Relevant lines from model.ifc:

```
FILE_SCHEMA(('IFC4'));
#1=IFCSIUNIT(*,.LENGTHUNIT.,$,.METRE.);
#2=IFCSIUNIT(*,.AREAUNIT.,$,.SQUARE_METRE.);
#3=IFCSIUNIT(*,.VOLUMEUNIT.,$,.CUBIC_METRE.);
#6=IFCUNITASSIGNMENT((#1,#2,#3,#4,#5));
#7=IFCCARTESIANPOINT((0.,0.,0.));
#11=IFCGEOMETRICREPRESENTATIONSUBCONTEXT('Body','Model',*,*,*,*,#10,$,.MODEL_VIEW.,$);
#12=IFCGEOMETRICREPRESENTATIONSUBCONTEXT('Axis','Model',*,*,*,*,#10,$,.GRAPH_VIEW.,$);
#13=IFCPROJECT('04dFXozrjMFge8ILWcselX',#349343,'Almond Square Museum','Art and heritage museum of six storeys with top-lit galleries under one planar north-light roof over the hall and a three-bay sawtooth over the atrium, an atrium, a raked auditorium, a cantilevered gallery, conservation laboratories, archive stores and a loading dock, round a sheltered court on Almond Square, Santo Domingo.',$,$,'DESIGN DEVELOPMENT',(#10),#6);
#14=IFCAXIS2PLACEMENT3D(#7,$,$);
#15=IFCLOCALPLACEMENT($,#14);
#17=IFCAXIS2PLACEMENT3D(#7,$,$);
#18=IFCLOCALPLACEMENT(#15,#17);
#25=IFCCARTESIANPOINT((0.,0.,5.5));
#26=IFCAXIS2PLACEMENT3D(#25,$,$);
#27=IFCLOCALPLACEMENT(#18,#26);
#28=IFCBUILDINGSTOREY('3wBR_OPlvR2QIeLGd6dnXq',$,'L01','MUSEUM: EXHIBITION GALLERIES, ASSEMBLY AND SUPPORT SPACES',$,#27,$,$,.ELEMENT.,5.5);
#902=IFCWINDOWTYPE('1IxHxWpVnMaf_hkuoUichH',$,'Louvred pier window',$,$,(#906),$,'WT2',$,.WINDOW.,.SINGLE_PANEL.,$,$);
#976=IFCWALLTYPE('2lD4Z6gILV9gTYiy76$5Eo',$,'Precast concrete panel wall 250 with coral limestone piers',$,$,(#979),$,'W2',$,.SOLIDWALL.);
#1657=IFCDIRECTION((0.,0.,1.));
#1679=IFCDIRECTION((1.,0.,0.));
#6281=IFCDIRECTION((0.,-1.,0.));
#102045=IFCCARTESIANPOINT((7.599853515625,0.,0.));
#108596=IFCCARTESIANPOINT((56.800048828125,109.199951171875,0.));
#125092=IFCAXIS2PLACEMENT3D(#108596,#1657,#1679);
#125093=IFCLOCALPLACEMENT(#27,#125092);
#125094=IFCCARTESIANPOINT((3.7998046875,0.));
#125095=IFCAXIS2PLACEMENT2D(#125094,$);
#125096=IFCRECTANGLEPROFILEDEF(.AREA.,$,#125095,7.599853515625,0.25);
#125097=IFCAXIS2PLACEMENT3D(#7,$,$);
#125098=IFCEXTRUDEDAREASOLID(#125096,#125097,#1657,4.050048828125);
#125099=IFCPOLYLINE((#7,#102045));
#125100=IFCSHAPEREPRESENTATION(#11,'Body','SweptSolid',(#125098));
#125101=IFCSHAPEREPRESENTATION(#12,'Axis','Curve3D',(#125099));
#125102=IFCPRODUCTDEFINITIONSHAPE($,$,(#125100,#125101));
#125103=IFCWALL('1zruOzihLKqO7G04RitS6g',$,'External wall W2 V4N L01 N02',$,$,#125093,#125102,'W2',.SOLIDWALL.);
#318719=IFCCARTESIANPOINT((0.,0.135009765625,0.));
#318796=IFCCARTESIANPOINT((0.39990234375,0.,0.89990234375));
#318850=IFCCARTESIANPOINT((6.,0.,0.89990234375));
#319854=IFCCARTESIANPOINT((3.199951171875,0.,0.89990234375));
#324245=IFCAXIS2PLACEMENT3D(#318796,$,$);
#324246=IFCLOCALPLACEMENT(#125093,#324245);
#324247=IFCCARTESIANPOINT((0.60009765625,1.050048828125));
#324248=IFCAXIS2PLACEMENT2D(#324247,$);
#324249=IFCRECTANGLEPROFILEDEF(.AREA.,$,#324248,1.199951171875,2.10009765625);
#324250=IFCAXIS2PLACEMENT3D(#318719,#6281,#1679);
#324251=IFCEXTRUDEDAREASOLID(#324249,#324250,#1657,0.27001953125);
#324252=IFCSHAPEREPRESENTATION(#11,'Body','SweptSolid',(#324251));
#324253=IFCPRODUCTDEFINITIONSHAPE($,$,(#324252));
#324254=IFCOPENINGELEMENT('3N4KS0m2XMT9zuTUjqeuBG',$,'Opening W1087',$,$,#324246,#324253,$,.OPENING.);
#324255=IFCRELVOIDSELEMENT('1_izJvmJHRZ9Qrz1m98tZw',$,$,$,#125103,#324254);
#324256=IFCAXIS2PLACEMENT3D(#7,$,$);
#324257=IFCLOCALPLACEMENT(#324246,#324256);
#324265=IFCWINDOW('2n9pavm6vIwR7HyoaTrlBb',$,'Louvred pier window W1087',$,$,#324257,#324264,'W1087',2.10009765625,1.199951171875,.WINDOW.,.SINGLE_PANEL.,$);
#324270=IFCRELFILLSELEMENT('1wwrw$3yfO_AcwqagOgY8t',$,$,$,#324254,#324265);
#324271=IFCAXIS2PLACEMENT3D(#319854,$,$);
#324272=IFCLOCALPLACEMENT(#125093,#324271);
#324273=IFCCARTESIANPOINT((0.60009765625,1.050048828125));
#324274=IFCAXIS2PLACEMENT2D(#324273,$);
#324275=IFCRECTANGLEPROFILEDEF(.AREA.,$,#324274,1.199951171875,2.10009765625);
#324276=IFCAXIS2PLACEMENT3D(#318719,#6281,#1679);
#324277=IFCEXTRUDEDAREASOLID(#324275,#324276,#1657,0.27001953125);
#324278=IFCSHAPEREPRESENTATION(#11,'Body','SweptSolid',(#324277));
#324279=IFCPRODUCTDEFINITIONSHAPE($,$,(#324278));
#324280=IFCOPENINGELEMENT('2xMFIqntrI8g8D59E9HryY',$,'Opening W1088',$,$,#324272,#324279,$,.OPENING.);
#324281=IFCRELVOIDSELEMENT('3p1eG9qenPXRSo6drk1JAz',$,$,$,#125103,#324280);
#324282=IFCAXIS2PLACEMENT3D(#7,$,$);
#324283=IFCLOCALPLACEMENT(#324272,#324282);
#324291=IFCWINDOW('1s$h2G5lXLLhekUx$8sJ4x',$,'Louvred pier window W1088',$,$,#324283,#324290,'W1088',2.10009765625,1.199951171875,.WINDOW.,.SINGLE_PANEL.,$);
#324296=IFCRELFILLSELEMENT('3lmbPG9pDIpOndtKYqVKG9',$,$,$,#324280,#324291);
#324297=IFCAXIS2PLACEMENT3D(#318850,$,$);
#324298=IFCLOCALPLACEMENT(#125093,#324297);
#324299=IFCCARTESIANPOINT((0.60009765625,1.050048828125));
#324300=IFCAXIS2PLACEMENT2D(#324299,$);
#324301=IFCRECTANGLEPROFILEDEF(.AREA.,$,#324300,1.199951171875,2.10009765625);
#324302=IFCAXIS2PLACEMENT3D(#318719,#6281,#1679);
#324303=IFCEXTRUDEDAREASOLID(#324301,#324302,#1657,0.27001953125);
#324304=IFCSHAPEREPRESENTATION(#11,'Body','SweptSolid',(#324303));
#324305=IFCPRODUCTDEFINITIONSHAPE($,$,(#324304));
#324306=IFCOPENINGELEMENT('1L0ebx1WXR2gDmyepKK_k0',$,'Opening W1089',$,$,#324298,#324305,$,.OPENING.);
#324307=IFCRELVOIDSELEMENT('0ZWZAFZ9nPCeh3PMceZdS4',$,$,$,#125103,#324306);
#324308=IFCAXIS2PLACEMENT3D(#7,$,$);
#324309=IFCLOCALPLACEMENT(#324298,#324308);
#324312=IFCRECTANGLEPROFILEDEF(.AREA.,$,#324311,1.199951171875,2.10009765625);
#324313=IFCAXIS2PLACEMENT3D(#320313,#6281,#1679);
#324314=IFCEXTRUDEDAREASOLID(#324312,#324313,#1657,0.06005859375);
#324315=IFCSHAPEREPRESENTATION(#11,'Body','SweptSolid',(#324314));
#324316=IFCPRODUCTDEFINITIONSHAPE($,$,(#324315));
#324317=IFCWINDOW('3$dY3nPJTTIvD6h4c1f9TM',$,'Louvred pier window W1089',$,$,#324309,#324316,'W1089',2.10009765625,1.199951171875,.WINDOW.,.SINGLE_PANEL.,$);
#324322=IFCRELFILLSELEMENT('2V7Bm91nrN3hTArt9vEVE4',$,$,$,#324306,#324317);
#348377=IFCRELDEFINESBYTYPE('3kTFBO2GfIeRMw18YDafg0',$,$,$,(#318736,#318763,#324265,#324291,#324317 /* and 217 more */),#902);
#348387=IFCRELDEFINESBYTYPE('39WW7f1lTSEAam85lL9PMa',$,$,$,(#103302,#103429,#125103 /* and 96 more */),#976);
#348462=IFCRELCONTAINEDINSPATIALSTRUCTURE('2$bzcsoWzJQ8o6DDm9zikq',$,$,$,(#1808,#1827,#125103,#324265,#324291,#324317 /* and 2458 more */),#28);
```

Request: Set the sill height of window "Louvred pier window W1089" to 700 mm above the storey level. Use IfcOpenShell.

```python
import numpy as np
import ifcopenshell
import ifcopenshell.api.geometry
import ifcopenshell.geom
import ifcopenshell.util.element
import ifcopenshell.util.placement
import ifcopenshell.util.shape
import ifcopenshell.util.unit

model = ifcopenshell.open("model.ifc")
unit_scale = ifcopenshell.util.unit.calculate_unit_scale(model)

window = model.by_id(324317)
opening = window.FillsVoids[0].RelatingOpeningElement
storey = ifcopenshell.util.element.get_container(window, ifc_class="IfcBuildingStorey")
level = ifcopenshell.util.placement.get_local_placement(storey.ObjectPlacement)[2, 3]

# The opening's origin need not be at the sill, so measure its lowest point.
shape = ifcopenshell.geom.create_shape(ifcopenshell.geom.settings(), opening)
bottom = ifcopenshell.util.shape.get_shape_bottom_elevation(shape, shape.geometry) / unit_scale
dz = level + 0.7 / unit_scale - bottom

shift = np.array([0.0, 0.0, dz])
# The window is placed relative to its opening, so it follows when the opening moves.
matrix = ifcopenshell.util.placement.get_local_placement(opening.ObjectPlacement)
matrix[:3, 3] += shift
ifcopenshell.api.geometry.edit_object_placement(
    model, product=opening, matrix=matrix, is_si=False, should_transform_children=True
)

print(f"moved by {dz * unit_scale:+.3f} m")

model.write("model-out.ifc")
```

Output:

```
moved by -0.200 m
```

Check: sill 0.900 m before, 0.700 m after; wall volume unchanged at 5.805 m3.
